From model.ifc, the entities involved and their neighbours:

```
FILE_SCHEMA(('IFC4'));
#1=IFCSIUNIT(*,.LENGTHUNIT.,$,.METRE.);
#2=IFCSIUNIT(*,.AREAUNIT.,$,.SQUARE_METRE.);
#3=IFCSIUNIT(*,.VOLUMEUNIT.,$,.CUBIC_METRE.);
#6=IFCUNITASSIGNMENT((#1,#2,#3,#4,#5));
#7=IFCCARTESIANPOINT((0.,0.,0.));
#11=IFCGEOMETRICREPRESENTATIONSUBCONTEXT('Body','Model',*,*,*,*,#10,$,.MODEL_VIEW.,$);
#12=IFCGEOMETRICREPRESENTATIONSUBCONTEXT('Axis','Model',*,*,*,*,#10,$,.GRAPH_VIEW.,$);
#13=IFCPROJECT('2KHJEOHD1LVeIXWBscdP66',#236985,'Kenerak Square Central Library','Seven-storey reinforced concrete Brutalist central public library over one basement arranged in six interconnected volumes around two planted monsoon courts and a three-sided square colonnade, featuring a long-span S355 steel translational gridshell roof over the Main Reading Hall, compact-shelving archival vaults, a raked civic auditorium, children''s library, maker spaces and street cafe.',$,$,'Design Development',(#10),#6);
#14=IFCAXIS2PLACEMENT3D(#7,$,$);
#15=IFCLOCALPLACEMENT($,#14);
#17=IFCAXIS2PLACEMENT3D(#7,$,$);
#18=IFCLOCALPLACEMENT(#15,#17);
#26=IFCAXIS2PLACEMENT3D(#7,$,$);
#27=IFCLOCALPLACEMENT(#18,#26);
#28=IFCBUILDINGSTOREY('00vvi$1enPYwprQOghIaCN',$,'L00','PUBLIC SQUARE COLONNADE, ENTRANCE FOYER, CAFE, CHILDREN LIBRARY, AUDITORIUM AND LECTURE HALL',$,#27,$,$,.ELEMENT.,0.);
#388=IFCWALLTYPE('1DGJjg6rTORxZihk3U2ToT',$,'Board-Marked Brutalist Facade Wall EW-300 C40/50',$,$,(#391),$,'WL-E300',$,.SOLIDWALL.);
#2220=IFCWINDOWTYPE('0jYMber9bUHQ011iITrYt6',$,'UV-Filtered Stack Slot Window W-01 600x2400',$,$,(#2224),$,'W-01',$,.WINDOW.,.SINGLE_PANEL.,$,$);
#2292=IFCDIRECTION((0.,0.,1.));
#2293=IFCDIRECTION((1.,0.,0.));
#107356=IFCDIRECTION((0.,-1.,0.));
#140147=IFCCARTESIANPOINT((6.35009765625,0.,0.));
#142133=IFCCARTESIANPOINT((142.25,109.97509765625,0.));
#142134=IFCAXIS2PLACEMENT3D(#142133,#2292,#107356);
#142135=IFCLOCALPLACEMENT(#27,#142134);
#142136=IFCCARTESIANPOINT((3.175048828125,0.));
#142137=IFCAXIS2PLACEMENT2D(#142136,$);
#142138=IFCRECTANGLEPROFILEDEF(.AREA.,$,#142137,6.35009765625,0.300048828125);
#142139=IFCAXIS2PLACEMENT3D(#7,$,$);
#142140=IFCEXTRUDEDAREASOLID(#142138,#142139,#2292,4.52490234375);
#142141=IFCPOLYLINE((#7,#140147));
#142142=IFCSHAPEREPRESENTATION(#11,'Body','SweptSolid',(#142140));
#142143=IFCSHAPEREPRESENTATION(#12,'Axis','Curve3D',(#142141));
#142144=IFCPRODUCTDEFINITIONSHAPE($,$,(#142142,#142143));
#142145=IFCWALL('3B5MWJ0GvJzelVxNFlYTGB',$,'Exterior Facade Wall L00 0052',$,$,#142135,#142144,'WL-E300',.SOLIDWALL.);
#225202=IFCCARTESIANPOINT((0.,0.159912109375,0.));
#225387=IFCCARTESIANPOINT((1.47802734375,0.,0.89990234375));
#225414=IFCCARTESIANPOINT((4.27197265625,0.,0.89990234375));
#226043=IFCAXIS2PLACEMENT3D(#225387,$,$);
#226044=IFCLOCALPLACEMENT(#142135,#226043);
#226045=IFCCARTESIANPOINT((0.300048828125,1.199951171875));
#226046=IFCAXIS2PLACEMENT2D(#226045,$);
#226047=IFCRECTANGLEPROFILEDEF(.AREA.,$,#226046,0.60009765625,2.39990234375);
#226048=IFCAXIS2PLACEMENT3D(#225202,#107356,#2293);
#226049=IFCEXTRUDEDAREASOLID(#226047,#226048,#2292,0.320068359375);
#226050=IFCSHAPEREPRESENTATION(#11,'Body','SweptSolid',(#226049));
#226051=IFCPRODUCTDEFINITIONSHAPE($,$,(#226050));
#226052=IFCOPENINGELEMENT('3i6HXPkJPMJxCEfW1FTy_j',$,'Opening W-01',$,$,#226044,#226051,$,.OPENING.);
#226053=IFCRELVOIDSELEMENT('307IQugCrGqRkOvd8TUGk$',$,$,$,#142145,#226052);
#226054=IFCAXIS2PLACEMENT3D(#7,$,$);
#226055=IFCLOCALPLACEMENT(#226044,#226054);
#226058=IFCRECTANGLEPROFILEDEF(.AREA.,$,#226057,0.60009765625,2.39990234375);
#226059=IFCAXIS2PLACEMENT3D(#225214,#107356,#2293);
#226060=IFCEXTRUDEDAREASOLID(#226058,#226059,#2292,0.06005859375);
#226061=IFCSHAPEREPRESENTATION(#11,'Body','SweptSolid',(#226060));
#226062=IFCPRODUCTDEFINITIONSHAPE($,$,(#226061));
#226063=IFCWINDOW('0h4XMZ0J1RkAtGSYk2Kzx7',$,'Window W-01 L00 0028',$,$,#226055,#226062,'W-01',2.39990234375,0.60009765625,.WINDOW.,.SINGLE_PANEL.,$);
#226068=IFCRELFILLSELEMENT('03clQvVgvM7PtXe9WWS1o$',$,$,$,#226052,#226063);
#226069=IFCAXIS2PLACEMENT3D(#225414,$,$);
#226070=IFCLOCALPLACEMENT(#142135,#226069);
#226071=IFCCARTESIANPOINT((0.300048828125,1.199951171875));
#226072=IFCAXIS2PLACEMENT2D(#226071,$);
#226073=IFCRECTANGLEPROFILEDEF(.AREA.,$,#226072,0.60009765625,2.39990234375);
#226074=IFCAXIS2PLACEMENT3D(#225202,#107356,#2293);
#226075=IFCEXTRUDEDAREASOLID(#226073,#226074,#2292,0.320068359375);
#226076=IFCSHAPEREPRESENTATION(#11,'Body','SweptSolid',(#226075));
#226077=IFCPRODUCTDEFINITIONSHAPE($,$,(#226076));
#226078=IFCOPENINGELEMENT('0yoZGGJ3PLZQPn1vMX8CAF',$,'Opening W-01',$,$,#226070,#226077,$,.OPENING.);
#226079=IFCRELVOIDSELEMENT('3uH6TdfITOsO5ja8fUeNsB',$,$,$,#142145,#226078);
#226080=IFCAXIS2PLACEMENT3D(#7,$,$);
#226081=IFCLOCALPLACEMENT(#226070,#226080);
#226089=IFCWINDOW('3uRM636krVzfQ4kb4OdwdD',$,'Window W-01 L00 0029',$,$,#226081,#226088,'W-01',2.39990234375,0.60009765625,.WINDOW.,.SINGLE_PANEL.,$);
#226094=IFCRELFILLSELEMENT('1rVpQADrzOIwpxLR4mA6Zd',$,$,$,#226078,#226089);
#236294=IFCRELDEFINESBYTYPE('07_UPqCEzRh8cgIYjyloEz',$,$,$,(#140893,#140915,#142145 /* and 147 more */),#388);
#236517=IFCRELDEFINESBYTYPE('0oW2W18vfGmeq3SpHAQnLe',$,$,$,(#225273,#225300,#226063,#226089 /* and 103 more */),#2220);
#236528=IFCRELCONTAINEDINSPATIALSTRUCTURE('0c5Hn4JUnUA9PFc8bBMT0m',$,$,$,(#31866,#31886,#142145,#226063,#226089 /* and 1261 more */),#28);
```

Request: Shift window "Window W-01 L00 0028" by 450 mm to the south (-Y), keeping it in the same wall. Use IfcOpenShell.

```python
import ifcopenshell
import ifcopenshell.api.geometry
import ifcopenshell.util.placement

model = ifcopenshell.open("model.ifc")

window = model.by_guid("0h4XMZ0J1RkAtGSYk2Kzx7")
opening = window.FillsVoids[0].RelatingOpeningElement
wall = opening.VoidsElements[0].RelatingBuildingElement

wall_matrix = ifcopenshell.util.placement.get_local_placement(wall.ObjectPlacement)
shift = wall_matrix[:3, 0] * 0.45
before = ifcopenshell.util.placement.get_local_placement(window.ObjectPlacement)[:3, 3].copy()

# The window is placed relative to its opening, so it follows when the opening moves.
matrix = ifcopenshell.util.placement.get_local_placement(opening.ObjectPlacement)
matrix[:3, 3] += shift
ifcopenshell.api.geometry.edit_object_placement(
    model, product=opening, matrix=matrix, is_si=False, should_transform_children=True
)

after = ifcopenshell.util.placement.get_local_placement(window.ObjectPlacement)[:3, 3]
print("window moved by", (after - before).round(3) + 0.0)

model.write("model_rev.ifc")
```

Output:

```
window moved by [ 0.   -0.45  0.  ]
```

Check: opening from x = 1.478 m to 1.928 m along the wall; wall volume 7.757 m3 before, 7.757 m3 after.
